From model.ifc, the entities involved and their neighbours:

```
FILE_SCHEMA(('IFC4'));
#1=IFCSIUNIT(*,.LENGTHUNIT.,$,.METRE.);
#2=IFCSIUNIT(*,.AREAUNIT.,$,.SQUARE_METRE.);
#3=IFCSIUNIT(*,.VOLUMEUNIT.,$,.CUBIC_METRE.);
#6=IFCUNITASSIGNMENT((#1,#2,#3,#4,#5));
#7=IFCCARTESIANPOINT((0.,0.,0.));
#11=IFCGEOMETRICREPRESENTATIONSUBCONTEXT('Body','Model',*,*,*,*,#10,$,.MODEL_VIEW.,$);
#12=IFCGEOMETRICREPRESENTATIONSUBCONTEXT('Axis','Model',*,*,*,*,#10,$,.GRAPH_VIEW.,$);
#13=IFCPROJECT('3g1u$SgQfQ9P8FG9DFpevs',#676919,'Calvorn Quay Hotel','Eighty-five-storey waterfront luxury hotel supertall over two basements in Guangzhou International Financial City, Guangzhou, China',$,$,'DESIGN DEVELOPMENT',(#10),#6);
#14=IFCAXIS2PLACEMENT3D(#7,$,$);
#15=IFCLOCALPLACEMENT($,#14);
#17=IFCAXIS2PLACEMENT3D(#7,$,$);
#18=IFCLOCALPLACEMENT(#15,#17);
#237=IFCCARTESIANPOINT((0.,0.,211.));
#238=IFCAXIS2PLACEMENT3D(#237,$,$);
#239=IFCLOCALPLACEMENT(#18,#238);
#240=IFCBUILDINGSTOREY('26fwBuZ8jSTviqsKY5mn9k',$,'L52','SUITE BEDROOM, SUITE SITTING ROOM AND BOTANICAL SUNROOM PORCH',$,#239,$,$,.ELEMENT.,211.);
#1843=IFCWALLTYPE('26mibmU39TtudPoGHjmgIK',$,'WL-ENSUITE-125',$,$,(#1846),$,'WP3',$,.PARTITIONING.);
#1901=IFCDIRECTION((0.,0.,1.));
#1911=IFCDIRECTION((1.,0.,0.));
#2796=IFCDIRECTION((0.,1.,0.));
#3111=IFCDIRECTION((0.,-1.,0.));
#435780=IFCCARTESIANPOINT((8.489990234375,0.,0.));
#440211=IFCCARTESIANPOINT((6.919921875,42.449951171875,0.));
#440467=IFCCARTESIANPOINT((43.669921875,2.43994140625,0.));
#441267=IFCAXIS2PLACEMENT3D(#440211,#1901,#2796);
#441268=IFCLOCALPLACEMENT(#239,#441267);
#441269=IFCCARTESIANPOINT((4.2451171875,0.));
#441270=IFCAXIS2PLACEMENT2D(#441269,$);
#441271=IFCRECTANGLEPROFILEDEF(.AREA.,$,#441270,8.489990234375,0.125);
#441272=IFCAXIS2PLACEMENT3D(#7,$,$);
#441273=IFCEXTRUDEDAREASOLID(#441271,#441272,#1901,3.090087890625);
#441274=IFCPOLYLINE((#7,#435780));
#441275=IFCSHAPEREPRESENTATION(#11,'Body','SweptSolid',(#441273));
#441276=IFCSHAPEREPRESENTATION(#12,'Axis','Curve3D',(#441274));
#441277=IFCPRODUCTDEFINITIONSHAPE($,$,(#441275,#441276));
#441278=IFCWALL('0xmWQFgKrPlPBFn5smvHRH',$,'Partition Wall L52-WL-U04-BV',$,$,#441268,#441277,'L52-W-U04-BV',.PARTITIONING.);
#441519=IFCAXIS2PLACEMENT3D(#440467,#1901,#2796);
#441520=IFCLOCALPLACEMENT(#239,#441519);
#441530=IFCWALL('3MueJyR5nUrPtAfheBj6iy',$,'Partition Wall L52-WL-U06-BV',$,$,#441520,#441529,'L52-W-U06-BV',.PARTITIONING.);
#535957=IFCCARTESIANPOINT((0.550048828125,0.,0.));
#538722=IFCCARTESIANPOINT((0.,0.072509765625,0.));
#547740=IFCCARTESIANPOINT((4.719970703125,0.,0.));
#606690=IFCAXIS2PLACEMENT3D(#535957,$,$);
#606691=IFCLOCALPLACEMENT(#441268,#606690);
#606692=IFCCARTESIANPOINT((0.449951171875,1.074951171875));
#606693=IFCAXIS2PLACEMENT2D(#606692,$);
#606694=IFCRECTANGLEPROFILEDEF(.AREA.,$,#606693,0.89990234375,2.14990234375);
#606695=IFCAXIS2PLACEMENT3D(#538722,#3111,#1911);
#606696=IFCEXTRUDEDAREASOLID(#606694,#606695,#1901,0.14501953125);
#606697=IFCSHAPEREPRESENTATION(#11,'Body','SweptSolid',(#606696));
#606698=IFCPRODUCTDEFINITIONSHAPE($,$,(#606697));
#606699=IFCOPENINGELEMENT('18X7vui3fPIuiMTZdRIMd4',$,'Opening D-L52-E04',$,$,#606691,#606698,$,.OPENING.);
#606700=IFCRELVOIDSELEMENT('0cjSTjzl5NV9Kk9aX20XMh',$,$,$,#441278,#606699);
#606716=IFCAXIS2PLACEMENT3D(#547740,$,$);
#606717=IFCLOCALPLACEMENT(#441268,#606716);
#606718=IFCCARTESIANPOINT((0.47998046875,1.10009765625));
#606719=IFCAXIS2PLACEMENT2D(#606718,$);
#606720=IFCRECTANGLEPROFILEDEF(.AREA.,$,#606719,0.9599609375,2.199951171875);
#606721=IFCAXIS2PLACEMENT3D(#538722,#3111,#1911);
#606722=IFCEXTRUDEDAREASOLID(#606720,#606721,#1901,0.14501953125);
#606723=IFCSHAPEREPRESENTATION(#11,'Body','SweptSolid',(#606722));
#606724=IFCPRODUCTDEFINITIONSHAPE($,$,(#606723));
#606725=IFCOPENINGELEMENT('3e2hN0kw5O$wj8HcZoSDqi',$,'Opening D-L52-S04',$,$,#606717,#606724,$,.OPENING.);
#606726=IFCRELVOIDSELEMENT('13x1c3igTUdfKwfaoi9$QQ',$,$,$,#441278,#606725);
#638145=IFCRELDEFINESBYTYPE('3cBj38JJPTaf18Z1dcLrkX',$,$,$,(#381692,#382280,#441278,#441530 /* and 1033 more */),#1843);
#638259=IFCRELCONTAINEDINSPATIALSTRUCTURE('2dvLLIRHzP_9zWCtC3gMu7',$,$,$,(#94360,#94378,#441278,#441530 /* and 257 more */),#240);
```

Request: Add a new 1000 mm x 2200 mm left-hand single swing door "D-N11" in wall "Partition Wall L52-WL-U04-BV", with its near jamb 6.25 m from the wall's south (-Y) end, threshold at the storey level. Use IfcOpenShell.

```python
import numpy as np
import ifcopenshell
import ifcopenshell.api.feature
import ifcopenshell.api.geometry
import ifcopenshell.api.root
import ifcopenshell.api.spatial
import ifcopenshell.geom
import ifcopenshell.util.element
import ifcopenshell.util.placement
import ifcopenshell.util.representation
import ifcopenshell.util.shape
import ifcopenshell.util.unit

model = ifcopenshell.open("model.ifc")
unit_scale = ifcopenshell.util.unit.calculate_unit_scale(model)
settings = ifcopenshell.geom.settings()


def volume(element):
    """Net volume in cubic metres, openings subtracted."""
    shape = ifcopenshell.geom.create_shape(settings, element)
    return ifcopenshell.util.shape.get_volume(shape.geometry)


wall = model.by_guid("0xmWQFgKrPlPBFn5smvHRH")
storey = ifcopenshell.util.element.get_container(wall, ifc_class="IfcBuildingStorey")
context = ifcopenshell.util.representation.get_context(model, "Model", "Body", "MODEL_VIEW")
before = volume(wall)

width, height, from_end, sill = 1, 2.2, 6.25, 0.0  # metres

# The wall runs along its own X axis, and the end named is its -X end.
wall_shape = ifcopenshell.geom.create_shape(settings, wall)
x, y, z = ifcopenshell.util.shape.get_vertices(wall_shape.geometry).T
start = x.min() + from_end
face, thickness = float(y.min()), float(y.max() - y.min())
wall_matrix = ifcopenshell.util.placement.get_local_placement(wall.ObjectPlacement)
level = ifcopenshell.util.placement.get_local_placement(storey.ObjectPlacement)[2, 3]


def in_wall(x, y):
    """Placement at x, y metres in the wall's axes, at sill height."""
    matrix = wall_matrix.copy()
    matrix[:, 3] = wall_matrix @ np.array([x / unit_scale, y / unit_scale, 0.0, 1.0])
    matrix[2, 3] = level + sill / unit_scale
    return matrix


# Opening: a box that overshoots both wall faces by 50 mm.
opening = ifcopenshell.api.root.create_entity(model, ifc_class="IfcOpeningElement", predefined_type="OPENING")
box = ifcopenshell.api.geometry.add_wall_representation(
    model, context=context, length=width, height=height, thickness=thickness + 0.1
)
ifcopenshell.api.geometry.assign_representation(model, product=opening, representation=box)
ifcopenshell.api.geometry.edit_object_placement(model, product=opening, matrix=in_wall(start, face - 0.05), is_si=False)
ifcopenshell.api.feature.add_feature(model, feature=opening, element=wall)

door = ifcopenshell.api.root.create_entity(model, ifc_class="IfcDoor", name="D-N11", predefined_type="DOOR")
door.OverallWidth, door.OverallHeight = width / unit_scale, height / unit_scale
door.OperationType = "SINGLE_SWING_LEFT"
body = ifcopenshell.api.geometry.add_door_representation(
    model,
    context=context,
    overall_width=door.OverallWidth,
    overall_height=door.OverallHeight,
    operation_type="SINGLE_SWING_LEFT",
    lining_properties={"LiningDepth": thickness / unit_scale, "ThresholdDepth": thickness / unit_scale},
)
ifcopenshell.api.geometry.assign_representation(model, product=door, representation=body)
ifcopenshell.api.spatial.assign_container(model, products=[door], relating_structure=storey)
ifcopenshell.api.feature.add_filling(model, opening=opening, element=door)

# The lining spans the wall, so the door starts at the wall face.
ifcopenshell.api.geometry.edit_object_placement(model, product=door, matrix=in_wall(start, face), is_si=False)

after = volume(wall)

print(f"wall volume {before:.3f} -> {after:.3f} m3")

model.write("model-out.ifc")
```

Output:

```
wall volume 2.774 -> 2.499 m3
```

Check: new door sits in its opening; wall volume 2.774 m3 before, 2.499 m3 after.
